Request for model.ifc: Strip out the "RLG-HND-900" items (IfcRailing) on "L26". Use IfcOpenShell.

First a look at what the model holds.

```python
import ifcopenshell
import ifcopenshell.util.element

model = ifcopenshell.open("model.ifc")
print(model.schema)
storey = next(s for s in model.by_type("IfcBuildingStorey") if s.Name == "L26")
railings = [e for e in ifcopenshell.util.element.get_decomposition(storey) if e.is_a("IfcRailing")]
seen = {}
for e in railings:
    element_type = ifcopenshell.util.element.get_type(e)
    name = element_type.Name if element_type not in (None, e) else None
    seen[name] = seen.get(name, 0) + 1
for name, count in sorted(seen.items(), key=str):
    print(count, "x", name)
```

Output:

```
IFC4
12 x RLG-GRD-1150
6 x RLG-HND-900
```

```python
import ifcopenshell
import ifcopenshell.api.root
import ifcopenshell.util.element

model = ifcopenshell.open("model.ifc")

storey = next(s for s in model.by_type("IfcBuildingStorey") if s.Name == "L26")
railings = [e for e in ifcopenshell.util.element.get_decomposition(storey) if e.is_a("IfcRailing")]
targets = [e for e in railings if (t := ifcopenshell.util.element.get_type(e)) not in (None, e) and t.Name == "RLG-HND-900"]

for e in targets:
    ifcopenshell.api.root.remove_product(model, product=e)
print(len(targets), "removed")

model.write("model_edited.ifc")
```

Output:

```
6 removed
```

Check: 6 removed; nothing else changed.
